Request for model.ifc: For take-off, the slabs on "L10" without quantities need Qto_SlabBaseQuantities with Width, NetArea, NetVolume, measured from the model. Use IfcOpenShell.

First a look at what the model holds.

```python
import ifcopenshell
import ifcopenshell.util.element
import ifcopenshell.util.unit

model = ifcopenshell.open("model.ifc")
print(model.schema)
for unit_type in ("LENGTHUNIT", "AREAUNIT", "VOLUMEUNIT"):
    print(unit_type, ifcopenshell.util.unit.calculate_unit_scale(model, unit_type))
storey = next(s for s in model.by_type("IfcBuildingStorey") if s.Name == "L10")
slabs = [e for e in ifcopenshell.util.element.get_decomposition(storey) if e.is_a("IfcSlab")]
for e in sorted(slabs, key=lambda e: e.id()):
    print(e.id(), e.is_a(), e.Name, list(ifcopenshell.util.element.get_psets(e, qtos_only=True)), sep=" | ")
```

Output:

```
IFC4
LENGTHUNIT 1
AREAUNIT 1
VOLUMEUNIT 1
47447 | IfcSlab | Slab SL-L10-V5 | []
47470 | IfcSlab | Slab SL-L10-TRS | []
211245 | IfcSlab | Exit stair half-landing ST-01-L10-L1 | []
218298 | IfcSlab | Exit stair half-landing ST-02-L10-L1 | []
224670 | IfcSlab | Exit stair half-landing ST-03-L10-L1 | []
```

```python
import ifcopenshell
import ifcopenshell.api.pset
import ifcopenshell.geom
import ifcopenshell.util.element
import ifcopenshell.util.shape
import ifcopenshell.util.unit

model = ifcopenshell.open("model.ifc")
unit_scale = ifcopenshell.util.unit.calculate_unit_scale(model)
area_scale = ifcopenshell.util.unit.calculate_unit_scale(model, "AREAUNIT")
volume_scale = ifcopenshell.util.unit.calculate_unit_scale(model, "VOLUMEUNIT")
settings = ifcopenshell.geom.settings()

storey = next(s for s in model.by_type("IfcBuildingStorey") if s.Name == "L10")
slabs = [e for e in ifcopenshell.util.element.get_decomposition(storey) if e.is_a("IfcSlab")]

for e in sorted(slabs, key=lambda e: e.id()):
    if ifcopenshell.util.element.get_psets(e, qtos_only=True, should_inherit=False):
        continue
    # Geometry comes back in metres, in the element's own axes.
    shape = ifcopenshell.geom.create_shape(settings, e)
    values = {
        "Width": ifcopenshell.util.shape.get_z(shape.geometry) / unit_scale,
        "NetArea": ifcopenshell.util.shape.get_footprint_area(shape.geometry) / area_scale,
        "NetVolume": ifcopenshell.util.shape.get_volume(shape.geometry) / volume_scale,
    }
    qto = ifcopenshell.api.pset.add_qto(model, product=e, name="Qto_SlabBaseQuantities")
    ifcopenshell.api.pset.edit_qto(model, qto=qto, properties=values)
    print(e.id(), {k: round(v, 3) for k, v in values.items()})

model.write("model_v2.ifc")
```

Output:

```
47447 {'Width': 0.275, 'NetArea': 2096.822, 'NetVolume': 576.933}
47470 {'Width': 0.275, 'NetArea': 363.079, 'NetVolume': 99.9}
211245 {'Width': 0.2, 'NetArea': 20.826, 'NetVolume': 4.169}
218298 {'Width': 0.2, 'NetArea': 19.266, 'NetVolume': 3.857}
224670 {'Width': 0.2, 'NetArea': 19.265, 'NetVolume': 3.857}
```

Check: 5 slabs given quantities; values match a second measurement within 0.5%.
